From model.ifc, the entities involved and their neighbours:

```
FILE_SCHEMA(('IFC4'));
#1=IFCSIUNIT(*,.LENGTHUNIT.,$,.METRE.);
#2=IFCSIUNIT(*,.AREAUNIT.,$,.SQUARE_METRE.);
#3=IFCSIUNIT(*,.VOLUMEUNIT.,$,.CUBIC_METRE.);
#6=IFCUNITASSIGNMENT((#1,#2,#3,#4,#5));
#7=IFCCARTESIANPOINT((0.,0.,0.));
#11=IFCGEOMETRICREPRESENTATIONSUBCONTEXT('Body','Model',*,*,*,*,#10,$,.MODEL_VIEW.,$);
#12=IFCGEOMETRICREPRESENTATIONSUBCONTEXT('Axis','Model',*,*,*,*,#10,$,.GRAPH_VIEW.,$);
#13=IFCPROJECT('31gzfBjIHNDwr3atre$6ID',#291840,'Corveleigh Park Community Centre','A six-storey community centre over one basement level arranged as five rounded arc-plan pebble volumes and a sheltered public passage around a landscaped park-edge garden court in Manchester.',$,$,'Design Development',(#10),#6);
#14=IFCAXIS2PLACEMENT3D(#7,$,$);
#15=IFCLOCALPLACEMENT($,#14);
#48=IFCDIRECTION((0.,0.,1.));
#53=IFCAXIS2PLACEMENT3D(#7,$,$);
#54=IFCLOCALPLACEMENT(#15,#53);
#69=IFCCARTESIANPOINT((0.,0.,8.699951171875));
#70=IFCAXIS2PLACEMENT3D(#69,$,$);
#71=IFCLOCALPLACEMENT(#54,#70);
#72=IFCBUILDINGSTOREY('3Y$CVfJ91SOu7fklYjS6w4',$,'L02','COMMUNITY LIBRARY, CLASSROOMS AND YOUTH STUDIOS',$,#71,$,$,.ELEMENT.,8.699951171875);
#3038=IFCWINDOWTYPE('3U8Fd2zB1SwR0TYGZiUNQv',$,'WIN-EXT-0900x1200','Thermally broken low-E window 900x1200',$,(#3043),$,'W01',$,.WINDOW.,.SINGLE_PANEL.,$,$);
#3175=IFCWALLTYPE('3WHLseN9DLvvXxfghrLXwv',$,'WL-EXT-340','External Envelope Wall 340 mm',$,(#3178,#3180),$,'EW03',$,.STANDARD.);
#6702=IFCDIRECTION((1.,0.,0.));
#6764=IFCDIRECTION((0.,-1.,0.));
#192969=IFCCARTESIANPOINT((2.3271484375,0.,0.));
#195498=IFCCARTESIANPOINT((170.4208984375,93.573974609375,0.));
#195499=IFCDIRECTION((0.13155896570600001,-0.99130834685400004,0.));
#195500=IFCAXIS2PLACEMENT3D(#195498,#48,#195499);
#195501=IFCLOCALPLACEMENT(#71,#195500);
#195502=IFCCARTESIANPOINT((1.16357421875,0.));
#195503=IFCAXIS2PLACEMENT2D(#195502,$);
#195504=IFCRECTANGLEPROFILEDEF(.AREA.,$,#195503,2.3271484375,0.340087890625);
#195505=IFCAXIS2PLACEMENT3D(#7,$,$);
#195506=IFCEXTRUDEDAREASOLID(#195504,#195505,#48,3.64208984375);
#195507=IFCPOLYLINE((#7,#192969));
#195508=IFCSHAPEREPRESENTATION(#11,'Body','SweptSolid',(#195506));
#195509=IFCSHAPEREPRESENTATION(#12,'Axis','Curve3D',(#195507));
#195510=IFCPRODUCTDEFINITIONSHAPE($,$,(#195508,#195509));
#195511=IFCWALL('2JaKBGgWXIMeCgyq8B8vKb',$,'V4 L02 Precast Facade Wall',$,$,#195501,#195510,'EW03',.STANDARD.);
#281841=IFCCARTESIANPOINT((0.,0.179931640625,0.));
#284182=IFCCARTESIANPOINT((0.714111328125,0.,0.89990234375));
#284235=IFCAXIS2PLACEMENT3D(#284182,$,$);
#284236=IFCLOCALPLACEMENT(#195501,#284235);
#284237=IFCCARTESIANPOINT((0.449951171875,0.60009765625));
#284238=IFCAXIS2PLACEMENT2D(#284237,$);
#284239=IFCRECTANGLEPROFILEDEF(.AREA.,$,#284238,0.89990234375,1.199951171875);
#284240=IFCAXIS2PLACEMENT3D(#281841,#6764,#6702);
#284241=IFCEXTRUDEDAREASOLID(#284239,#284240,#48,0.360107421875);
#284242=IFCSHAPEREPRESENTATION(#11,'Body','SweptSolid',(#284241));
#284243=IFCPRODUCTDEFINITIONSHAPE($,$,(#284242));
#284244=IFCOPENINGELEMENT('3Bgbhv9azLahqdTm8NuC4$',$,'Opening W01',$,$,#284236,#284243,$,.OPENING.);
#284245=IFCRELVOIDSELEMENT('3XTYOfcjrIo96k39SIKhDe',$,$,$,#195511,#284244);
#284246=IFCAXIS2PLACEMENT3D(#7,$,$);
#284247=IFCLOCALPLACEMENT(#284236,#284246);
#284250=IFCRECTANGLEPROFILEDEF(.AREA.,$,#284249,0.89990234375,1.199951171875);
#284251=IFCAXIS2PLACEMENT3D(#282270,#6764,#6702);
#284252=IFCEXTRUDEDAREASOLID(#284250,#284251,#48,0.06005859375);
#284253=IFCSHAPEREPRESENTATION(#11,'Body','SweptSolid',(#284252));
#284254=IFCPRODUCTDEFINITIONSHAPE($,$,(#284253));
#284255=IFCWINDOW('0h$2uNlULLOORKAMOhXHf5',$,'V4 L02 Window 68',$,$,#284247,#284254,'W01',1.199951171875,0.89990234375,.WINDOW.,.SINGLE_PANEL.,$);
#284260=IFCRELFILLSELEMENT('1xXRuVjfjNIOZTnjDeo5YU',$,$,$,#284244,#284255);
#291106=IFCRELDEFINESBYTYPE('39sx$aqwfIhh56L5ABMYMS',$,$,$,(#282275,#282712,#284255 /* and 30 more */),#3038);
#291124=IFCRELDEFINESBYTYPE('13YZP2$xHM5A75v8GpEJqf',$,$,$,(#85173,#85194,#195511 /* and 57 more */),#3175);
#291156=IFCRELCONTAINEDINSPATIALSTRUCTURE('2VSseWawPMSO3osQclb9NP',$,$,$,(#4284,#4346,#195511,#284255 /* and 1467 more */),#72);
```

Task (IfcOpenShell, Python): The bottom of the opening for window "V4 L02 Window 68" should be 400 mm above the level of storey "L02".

```python
import numpy as np
import ifcopenshell
import ifcopenshell.api.geometry
import ifcopenshell.geom
import ifcopenshell.util.element
import ifcopenshell.util.placement
import ifcopenshell.util.shape
import ifcopenshell.util.unit

model = ifcopenshell.open("model.ifc")
unit_scale = ifcopenshell.util.unit.calculate_unit_scale(model)

window = model.by_guid("0h$2uNlULLOORKAMOhXHf5")
opening = window.FillsVoids[0].RelatingOpeningElement
storey = ifcopenshell.util.element.get_container(window, ifc_class="IfcBuildingStorey")
level = ifcopenshell.util.placement.get_local_placement(storey.ObjectPlacement)[2, 3]

# The opening's origin need not be at the sill, so measure its lowest point.
shape = ifcopenshell.geom.create_shape(ifcopenshell.geom.settings(), opening)
bottom = ifcopenshell.util.shape.get_shape_bottom_elevation(shape, shape.geometry) / unit_scale
dz = level + 0.4 - bottom

shift = np.array([0.0, 0.0, dz])
# The window is placed relative to its opening, so it follows when the opening moves.
matrix = ifcopenshell.util.placement.get_local_placement(opening.ObjectPlacement)
matrix[:3, 3] += shift
ifcopenshell.api.geometry.edit_object_placement(
    model, product=opening, matrix=matrix, is_si=False, should_transform_children=True
)

print(f"moved by {dz * unit_scale:+.3f} m")

model.write("model_v2.ifc")
```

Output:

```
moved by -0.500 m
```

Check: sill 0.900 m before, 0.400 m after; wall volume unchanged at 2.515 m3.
